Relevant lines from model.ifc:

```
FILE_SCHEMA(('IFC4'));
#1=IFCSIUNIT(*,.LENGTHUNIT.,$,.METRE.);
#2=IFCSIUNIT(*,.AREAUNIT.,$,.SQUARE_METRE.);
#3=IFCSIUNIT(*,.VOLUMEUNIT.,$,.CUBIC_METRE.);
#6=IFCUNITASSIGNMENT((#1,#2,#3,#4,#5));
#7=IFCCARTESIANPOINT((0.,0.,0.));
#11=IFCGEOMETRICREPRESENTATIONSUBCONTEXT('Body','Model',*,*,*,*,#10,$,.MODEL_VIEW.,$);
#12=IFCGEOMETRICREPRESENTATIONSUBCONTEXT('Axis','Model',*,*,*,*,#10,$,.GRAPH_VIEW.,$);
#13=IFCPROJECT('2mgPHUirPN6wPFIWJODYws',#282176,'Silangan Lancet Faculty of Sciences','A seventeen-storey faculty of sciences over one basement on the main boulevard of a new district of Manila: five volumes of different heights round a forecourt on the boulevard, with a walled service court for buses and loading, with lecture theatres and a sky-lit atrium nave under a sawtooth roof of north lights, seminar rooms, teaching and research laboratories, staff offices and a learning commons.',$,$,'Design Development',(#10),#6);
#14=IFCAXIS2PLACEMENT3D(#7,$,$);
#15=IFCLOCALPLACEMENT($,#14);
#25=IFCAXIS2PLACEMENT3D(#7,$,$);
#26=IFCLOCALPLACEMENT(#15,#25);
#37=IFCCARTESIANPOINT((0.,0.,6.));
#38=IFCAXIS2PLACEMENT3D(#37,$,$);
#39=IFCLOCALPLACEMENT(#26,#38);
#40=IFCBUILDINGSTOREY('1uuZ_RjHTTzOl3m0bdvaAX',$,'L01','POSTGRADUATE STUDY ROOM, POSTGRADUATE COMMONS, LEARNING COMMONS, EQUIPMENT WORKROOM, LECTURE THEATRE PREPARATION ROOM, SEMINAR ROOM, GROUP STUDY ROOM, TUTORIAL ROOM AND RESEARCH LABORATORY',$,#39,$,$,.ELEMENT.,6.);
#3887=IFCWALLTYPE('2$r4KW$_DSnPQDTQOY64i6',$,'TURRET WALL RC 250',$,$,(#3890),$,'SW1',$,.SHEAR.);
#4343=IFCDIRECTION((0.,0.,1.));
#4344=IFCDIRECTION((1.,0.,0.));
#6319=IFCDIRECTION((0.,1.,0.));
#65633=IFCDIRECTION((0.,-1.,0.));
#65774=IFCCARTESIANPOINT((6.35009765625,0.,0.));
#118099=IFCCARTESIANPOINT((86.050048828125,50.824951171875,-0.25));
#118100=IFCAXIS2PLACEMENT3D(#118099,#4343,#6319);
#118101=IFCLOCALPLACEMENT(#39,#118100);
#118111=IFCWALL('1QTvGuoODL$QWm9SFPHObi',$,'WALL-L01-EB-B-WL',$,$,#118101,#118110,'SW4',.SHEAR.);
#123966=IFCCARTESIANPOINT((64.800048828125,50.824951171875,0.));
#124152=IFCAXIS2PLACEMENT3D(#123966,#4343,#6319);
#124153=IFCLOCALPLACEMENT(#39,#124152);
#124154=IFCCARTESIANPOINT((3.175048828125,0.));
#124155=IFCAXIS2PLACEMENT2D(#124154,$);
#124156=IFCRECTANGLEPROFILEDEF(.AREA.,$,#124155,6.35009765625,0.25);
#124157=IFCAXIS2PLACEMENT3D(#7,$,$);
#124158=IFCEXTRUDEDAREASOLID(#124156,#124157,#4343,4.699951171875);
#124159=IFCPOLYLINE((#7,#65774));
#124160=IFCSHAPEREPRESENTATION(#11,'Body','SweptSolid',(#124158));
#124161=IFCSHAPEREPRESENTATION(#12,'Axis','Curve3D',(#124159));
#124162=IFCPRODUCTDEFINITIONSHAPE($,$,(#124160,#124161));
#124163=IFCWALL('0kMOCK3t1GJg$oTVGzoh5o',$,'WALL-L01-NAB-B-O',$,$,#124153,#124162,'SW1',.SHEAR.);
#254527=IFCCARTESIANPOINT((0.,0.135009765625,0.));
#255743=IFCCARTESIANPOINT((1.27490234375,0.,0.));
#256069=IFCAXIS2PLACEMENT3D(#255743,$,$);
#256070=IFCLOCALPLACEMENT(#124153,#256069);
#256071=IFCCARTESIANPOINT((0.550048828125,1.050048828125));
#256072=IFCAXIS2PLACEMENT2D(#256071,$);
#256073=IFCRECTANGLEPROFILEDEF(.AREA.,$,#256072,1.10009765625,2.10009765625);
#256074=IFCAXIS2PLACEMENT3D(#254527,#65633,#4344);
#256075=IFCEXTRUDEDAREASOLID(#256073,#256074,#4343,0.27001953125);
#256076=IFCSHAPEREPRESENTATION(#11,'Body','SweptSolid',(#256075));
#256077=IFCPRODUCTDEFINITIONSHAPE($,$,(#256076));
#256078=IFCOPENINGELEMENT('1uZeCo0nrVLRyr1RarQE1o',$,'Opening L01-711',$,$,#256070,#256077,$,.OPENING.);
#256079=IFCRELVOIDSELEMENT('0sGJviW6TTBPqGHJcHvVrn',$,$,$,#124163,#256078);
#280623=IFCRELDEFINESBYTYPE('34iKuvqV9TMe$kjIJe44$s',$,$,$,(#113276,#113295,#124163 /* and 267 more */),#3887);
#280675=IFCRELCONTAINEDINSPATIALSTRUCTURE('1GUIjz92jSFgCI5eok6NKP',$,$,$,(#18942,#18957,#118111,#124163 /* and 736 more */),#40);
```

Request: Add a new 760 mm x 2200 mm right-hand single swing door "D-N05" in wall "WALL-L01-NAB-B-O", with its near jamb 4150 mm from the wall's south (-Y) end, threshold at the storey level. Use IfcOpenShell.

```python
import numpy as np
import ifcopenshell
import ifcopenshell.api.feature
import ifcopenshell.api.geometry
import ifcopenshell.api.root
import ifcopenshell.api.spatial
import ifcopenshell.geom
import ifcopenshell.util.element
import ifcopenshell.util.placement
import ifcopenshell.util.representation
import ifcopenshell.util.shape
import ifcopenshell.util.unit

model = ifcopenshell.open("model.ifc")
unit_scale = ifcopenshell.util.unit.calculate_unit_scale(model)
settings = ifcopenshell.geom.settings()


def volume(element):
    """Net volume in cubic metres, openings subtracted."""
    shape = ifcopenshell.geom.create_shape(settings, element)
    return ifcopenshell.util.shape.get_volume(shape.geometry)


wall = model.by_guid("0kMOCK3t1GJg$oTVGzoh5o")
storey = ifcopenshell.util.element.get_container(wall, ifc_class="IfcBuildingStorey")
context = ifcopenshell.util.representation.get_context(model, "Model", "Body", "MODEL_VIEW")
before = volume(wall)

width, height, from_end, sill = 0.76, 2.2, 4.15, 0.0  # metres

# The wall runs along its own X axis, and the end named is its -X end.
wall_shape = ifcopenshell.geom.create_shape(settings, wall)
x, y, z = ifcopenshell.util.shape.get_vertices(wall_shape.geometry).T
start = x.min() + from_end
face, thickness = float(y.min()), float(y.max() - y.min())
wall_matrix = ifcopenshell.util.placement.get_local_placement(wall.ObjectPlacement)
level = ifcopenshell.util.placement.get_local_placement(storey.ObjectPlacement)[2, 3]


def in_wall(x, y):
    """Placement at x, y metres in the wall's axes, at sill height."""
    matrix = wall_matrix.copy()
    matrix[:, 3] = wall_matrix @ np.array([x / unit_scale, y / unit_scale, 0.0, 1.0])
    matrix[2, 3] = level + sill / unit_scale
    return matrix


# Opening: a box that overshoots both wall faces by 50 mm.
opening = ifcopenshell.api.root.create_entity(model, ifc_class="IfcOpeningElement", predefined_type="OPENING")
box = ifcopenshell.api.geometry.add_wall_representation(
    model, context=context, length=width, height=height, thickness=thickness + 0.1
)
ifcopenshell.api.geometry.assign_representation(model, product=opening, representation=box)
ifcopenshell.api.geometry.edit_object_placement(model, product=opening, matrix=in_wall(start, face - 0.05), is_si=False)
ifcopenshell.api.feature.add_feature(model, feature=opening, element=wall)

door = ifcopenshell.api.root.create_entity(model, ifc_class="IfcDoor", name="D-N05", predefined_type="DOOR")
door.OverallWidth, door.OverallHeight = width / unit_scale, height / unit_scale
door.OperationType = "SINGLE_SWING_RIGHT"
body = ifcopenshell.api.geometry.add_door_representation(
    model,
    context=context,
    overall_width=door.OverallWidth,
    overall_height=door.OverallHeight,
    operation_type="SINGLE_SWING_RIGHT",
    lining_properties={"LiningDepth": thickness / unit_scale, "ThresholdDepth": thickness / unit_scale},
)
ifcopenshell.api.geometry.assign_representation(model, product=door, representation=body)
ifcopenshell.api.spatial.assign_container(model, products=[door], relating_structure=storey)
ifcopenshell.api.feature.add_filling(model, opening=opening, element=door)

# The lining spans the wall, so the door starts at the wall face.
ifcopenshell.api.geometry.edit_object_placement(model, product=door, matrix=in_wall(start, face), is_si=False)

after = volume(wall)

print(f"wall volume {before:.3f} -> {after:.3f} m3")

model.write("model_edited.ifc")
```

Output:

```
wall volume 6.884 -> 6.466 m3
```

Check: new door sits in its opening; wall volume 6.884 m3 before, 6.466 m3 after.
